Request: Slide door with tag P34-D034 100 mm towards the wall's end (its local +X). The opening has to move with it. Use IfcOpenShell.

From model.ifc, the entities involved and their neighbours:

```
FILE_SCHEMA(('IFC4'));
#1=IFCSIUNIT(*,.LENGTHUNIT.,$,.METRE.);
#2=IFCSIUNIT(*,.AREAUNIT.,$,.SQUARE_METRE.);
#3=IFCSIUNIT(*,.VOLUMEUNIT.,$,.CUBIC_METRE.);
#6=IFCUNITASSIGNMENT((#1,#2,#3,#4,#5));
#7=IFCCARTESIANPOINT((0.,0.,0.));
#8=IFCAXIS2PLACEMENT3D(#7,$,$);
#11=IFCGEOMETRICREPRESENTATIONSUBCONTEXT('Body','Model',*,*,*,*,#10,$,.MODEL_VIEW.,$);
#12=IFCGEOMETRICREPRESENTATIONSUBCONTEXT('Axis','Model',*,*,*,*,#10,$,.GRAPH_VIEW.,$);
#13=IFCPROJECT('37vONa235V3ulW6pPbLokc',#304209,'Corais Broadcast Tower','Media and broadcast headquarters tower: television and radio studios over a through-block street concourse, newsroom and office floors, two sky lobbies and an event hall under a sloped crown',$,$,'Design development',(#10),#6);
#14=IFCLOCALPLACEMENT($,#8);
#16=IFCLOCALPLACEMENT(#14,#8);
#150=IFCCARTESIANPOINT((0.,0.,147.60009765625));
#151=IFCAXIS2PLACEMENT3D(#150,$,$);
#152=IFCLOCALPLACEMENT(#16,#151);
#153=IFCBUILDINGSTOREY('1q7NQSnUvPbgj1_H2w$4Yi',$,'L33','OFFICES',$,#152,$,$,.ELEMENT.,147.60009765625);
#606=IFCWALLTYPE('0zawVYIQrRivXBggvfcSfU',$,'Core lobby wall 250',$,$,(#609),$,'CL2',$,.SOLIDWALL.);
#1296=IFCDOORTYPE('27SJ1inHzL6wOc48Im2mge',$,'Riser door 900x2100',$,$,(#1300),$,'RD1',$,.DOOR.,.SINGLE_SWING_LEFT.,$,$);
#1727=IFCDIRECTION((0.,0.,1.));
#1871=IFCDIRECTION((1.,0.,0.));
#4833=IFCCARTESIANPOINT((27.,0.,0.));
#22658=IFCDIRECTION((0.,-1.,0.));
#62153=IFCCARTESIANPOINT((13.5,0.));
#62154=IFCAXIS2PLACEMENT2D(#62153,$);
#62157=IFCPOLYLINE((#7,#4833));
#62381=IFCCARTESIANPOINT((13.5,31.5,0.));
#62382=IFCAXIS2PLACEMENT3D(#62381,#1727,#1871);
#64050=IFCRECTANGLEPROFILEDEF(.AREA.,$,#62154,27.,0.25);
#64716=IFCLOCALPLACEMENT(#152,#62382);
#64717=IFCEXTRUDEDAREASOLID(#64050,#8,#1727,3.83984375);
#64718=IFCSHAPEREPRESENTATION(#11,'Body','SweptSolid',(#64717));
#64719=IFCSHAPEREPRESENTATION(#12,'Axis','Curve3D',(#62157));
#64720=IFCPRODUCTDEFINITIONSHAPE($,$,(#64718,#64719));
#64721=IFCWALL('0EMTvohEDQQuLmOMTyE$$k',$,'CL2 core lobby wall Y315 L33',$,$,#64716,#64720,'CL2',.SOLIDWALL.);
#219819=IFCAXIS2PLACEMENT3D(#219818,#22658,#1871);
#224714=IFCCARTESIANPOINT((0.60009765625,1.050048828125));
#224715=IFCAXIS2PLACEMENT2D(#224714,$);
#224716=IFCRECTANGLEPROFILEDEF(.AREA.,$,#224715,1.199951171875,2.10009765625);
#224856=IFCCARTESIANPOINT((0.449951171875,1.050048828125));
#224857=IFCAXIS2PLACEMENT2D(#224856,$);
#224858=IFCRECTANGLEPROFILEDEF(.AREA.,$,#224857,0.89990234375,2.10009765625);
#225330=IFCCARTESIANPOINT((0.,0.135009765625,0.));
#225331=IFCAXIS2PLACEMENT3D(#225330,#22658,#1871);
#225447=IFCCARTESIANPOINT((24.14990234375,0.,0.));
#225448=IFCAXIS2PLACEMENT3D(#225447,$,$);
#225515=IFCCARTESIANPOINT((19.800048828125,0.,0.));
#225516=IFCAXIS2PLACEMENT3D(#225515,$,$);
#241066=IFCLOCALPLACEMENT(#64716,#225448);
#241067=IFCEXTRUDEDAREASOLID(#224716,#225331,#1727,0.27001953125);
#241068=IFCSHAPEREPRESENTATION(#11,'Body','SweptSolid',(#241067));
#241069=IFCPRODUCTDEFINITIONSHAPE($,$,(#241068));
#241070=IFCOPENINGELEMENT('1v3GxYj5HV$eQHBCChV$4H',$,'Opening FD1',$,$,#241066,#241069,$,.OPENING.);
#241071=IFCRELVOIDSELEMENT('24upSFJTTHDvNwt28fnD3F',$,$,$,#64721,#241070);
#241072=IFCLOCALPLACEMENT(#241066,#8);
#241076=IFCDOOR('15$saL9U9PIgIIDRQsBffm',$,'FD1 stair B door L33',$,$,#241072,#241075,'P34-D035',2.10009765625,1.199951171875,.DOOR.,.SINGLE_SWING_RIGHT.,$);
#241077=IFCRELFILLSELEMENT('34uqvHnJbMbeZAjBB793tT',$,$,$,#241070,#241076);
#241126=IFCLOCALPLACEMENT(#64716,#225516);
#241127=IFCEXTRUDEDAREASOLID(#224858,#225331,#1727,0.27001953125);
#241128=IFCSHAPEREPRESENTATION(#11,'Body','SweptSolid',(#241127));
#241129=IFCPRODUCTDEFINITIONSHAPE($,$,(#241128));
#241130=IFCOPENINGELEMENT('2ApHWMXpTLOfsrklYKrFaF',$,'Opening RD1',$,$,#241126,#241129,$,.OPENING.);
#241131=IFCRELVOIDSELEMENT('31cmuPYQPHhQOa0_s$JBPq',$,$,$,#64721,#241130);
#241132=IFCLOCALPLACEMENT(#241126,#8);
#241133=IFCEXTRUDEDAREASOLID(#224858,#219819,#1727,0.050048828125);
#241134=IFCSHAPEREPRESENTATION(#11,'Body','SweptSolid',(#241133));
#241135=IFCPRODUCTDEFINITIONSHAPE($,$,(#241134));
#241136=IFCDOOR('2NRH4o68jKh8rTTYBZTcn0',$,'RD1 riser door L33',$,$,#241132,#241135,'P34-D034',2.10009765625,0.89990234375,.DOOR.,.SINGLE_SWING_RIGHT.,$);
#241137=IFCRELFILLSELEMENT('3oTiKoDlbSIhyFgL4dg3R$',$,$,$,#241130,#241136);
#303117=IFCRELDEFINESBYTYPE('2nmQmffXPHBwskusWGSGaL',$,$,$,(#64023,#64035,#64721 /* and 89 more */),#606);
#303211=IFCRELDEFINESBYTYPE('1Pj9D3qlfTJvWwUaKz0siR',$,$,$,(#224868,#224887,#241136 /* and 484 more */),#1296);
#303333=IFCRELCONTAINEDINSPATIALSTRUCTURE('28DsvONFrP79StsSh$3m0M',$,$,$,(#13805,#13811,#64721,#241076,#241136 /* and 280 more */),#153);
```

```python
import ifcopenshell
import ifcopenshell.api.geometry
import ifcopenshell.util.placement
import ifcopenshell.util.unit

model = ifcopenshell.open("model.ifc")
unit_scale = ifcopenshell.util.unit.calculate_unit_scale(model)

door = model.by_guid("2NRH4o68jKh8rTTYBZTcn0")
opening = door.FillsVoids[0].RelatingOpeningElement
wall = opening.VoidsElements[0].RelatingBuildingElement

wall_matrix = ifcopenshell.util.placement.get_local_placement(wall.ObjectPlacement)
shift = wall_matrix[:3, 0] * 0.1 / unit_scale
before = ifcopenshell.util.placement.get_local_placement(door.ObjectPlacement)[:3, 3].copy()

# The door is placed relative to its opening, so it follows when the opening moves.
matrix = ifcopenshell.util.placement.get_local_placement(opening.ObjectPlacement)
matrix[:3, 3] += shift
ifcopenshell.api.geometry.edit_object_placement(
    model, product=opening, matrix=matrix, is_si=False, should_transform_children=True
)

after = ifcopenshell.util.placement.get_local_placement(door.ObjectPlacement)[:3, 3]
print("door moved by", (after - before).round(3) + 0.0)

model.write("model-out.ifc")
```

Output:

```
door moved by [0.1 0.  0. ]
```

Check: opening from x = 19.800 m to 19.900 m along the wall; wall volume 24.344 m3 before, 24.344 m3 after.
